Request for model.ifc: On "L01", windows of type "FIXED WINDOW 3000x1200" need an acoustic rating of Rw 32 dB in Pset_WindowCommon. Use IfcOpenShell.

First a look at what the model holds.

```python
import ifcopenshell
import ifcopenshell.util.element

model = ifcopenshell.open("model.ifc")
print(model.schema)
storey = next(s for s in model.by_type("IfcBuildingStorey") if s.Name == "L01")
windows = [e for e in ifcopenshell.util.element.get_decomposition(storey) if e.is_a("IfcWindow")]
seen = {}
for e in windows:
    element_type = ifcopenshell.util.element.get_type(e)
    key = (element_type.Name if element_type != e and element_type else None, ifcopenshell.util.element.get_pset(e, "Pset_WindowCommon", "AcousticRating"))
    seen[key] = seen.get(key, 0) + 1
for (name, value), count in sorted(seen.items(), key=str):
    print(count, "x", name, "|", value)
```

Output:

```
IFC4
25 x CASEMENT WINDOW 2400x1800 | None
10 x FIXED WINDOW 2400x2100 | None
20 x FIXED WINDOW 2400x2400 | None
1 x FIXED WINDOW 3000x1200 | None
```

```python
import ifcopenshell
import ifcopenshell.api.pset
import ifcopenshell.util.element

model = ifcopenshell.open("model.ifc")

storey = next(s for s in model.by_type("IfcBuildingStorey") if s.Name == "L01")
windows = [e for e in ifcopenshell.util.element.get_decomposition(storey) if e.is_a("IfcWindow")]

count = 0
for e in windows:
    element_type = ifcopenshell.util.element.get_type(e)
    if element_type in (None, e) or element_type.Name != "FIXED WINDOW 3000x1200":
        continue
    # add_pset returns the element's existing set when there is one.
    pset = ifcopenshell.api.pset.add_pset(model, product=e, name="Pset_WindowCommon")
    ifcopenshell.api.pset.edit_pset(model, pset=pset, properties={"AcousticRating": "Rw 32 dB"})
    count += 1

print(count, "windows updated")

model.write("model-out.ifc")
```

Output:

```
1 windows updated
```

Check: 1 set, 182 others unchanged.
